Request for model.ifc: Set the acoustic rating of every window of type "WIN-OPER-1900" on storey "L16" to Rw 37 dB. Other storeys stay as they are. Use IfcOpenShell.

First a look at what the model holds.

```python
import ifcopenshell
import ifcopenshell.util.element

model = ifcopenshell.open("model.ifc")
print(model.schema)
storey = next(s for s in model.by_type("IfcBuildingStorey") if s.Name == "L16")
windows = [e for e in ifcopenshell.util.element.get_decomposition(storey) if e.is_a("IfcWindow")]
seen = {}
for e in windows:
    element_type = ifcopenshell.util.element.get_type(e)
    key = (element_type.Name if element_type != e and element_type else None, ifcopenshell.util.element.get_pset(e, "Pset_WindowCommon", "AcousticRating"))
    seen[key] = seen.get(key, 0) + 1
for (name, value), count in sorted(seen.items(), key=str):
    print(count, "x", name, "|", value)
```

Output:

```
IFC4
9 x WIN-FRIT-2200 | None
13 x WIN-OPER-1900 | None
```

```python
import ifcopenshell
import ifcopenshell.api.pset
import ifcopenshell.util.element

model = ifcopenshell.open("model.ifc")

storey = next(s for s in model.by_type("IfcBuildingStorey") if s.Name == "L16")
windows = [e for e in ifcopenshell.util.element.get_decomposition(storey) if e.is_a("IfcWindow")]

count = 0
for e in windows:
    element_type = ifcopenshell.util.element.get_type(e)
    if element_type in (None, e) or element_type.Name != "WIN-OPER-1900":
        continue
    found = ifcopenshell.util.element.get_pset(e, "Pset_WindowCommon", should_inherit=False)
    if found:
        pset = model.by_id(found["id"])
        if len(ifcopenshell.util.element.get_elements_by_pset(pset)) > 1:
            pset = ifcopenshell.api.pset.unshare_pset(model, products=[e], pset=pset)[0]
    else:
        pset = ifcopenshell.api.pset.add_pset(model, product=e, name="Pset_WindowCommon")
    ifcopenshell.api.pset.edit_pset(model, pset=pset, properties={"AcousticRating": "Rw 37 dB"})
    count += 1

print(count, "windows updated")

model.write("model_edited.ifc")
```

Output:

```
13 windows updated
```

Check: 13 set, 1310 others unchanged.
